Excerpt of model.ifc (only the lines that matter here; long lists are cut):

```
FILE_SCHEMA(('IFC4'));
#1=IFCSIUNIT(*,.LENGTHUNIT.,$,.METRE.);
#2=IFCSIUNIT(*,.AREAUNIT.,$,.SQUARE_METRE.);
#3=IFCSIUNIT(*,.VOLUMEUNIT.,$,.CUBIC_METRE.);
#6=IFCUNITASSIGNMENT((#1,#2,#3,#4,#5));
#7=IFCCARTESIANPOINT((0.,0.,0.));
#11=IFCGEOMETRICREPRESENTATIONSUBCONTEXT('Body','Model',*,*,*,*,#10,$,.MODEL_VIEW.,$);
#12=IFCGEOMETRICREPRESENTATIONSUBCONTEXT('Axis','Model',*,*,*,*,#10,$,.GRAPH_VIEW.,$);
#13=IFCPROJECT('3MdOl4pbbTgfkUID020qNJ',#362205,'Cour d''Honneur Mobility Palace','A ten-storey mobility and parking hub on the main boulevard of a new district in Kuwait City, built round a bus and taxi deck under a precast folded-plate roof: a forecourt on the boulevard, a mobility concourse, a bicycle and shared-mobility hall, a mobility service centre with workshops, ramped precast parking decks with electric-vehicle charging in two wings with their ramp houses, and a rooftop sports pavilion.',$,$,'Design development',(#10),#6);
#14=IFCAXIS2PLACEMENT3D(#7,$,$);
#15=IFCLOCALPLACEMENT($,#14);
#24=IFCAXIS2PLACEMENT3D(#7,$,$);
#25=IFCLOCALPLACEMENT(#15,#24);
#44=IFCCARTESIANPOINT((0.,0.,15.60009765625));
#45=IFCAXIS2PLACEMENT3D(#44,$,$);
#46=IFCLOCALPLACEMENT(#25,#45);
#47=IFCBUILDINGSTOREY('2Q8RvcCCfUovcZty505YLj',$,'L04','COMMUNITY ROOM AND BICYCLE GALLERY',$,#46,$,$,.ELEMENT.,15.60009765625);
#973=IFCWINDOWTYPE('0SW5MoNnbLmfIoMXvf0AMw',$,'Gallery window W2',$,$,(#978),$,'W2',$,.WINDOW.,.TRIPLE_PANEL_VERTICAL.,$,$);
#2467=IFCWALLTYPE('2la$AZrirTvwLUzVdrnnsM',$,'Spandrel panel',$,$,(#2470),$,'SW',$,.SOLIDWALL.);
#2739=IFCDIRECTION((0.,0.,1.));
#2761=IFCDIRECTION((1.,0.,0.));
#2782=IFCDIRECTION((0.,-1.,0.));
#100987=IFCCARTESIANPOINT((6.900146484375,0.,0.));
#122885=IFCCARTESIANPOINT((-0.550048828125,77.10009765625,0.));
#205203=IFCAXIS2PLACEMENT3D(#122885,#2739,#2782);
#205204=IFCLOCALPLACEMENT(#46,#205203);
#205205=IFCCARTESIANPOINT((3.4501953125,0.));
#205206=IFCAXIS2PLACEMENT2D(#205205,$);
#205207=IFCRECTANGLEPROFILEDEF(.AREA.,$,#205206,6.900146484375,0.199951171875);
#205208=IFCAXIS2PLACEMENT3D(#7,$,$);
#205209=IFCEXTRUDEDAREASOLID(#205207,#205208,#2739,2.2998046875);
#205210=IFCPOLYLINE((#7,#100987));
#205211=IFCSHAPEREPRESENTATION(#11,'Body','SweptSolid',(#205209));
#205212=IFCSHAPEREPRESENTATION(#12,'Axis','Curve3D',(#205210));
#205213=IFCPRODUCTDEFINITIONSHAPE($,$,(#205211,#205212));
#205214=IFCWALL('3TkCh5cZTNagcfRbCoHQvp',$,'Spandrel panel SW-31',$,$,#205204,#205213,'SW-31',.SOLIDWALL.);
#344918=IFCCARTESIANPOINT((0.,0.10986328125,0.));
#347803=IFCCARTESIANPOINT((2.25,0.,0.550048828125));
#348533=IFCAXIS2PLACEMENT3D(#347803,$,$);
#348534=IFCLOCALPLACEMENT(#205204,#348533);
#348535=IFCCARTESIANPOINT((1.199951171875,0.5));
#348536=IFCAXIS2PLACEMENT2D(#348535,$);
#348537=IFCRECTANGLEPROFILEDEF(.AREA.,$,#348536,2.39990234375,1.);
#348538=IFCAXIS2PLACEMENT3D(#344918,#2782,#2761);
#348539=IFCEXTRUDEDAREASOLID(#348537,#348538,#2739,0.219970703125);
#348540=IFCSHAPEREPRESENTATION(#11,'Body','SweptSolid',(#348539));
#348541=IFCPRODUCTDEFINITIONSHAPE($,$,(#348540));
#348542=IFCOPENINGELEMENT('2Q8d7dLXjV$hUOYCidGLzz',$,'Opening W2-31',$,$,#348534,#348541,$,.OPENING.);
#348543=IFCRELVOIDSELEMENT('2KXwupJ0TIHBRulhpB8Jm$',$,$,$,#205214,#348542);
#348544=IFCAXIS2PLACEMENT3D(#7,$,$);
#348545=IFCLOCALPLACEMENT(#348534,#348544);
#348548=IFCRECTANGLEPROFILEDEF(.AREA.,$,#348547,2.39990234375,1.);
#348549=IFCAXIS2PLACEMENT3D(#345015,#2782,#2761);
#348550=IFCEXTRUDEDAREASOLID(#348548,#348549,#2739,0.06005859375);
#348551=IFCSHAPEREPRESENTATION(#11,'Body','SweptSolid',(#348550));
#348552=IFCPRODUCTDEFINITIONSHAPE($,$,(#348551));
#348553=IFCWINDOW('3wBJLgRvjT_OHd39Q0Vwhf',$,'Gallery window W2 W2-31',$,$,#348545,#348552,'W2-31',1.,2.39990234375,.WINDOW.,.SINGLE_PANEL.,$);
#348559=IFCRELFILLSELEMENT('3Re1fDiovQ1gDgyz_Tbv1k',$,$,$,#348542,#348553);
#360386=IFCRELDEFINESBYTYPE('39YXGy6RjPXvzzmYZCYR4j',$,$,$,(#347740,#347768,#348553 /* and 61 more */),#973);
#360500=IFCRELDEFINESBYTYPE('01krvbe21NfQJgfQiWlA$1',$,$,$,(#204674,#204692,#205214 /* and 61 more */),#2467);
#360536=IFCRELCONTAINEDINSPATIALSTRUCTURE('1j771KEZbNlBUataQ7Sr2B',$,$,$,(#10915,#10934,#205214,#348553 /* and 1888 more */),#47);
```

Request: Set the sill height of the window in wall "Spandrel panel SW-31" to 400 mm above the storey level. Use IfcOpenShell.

```python
import numpy as np
import ifcopenshell
import ifcopenshell.api.geometry
import ifcopenshell.geom
import ifcopenshell.util.element
import ifcopenshell.util.placement
import ifcopenshell.util.shape
import ifcopenshell.util.unit

model = ifcopenshell.open("model.ifc")
unit_scale = ifcopenshell.util.unit.calculate_unit_scale(model)

window = model.by_id(348553)
opening = window.FillsVoids[0].RelatingOpeningElement
storey = ifcopenshell.util.element.get_container(window, ifc_class="IfcBuildingStorey")
level = ifcopenshell.util.placement.get_local_placement(storey.ObjectPlacement)[2, 3]

# The opening's origin need not be at the sill, so measure its lowest point.
shape = ifcopenshell.geom.create_shape(ifcopenshell.geom.settings(), opening)
bottom = ifcopenshell.util.shape.get_shape_bottom_elevation(shape, shape.geometry) / unit_scale
dz = level + 0.4 / unit_scale - bottom

shift = np.array([0.0, 0.0, dz])
# The window is placed relative to its opening, so it follows when the opening moves.
matrix = ifcopenshell.util.placement.get_local_placement(opening.ObjectPlacement)
matrix[:3, 3] += shift
ifcopenshell.api.geometry.edit_object_placement(
    model, product=opening, matrix=matrix, is_si=False, should_transform_children=True
)

print(f"moved by {dz * unit_scale:+.3f} m")

model.write("model_edited.ifc")
```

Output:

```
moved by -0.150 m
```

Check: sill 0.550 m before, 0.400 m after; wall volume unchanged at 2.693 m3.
